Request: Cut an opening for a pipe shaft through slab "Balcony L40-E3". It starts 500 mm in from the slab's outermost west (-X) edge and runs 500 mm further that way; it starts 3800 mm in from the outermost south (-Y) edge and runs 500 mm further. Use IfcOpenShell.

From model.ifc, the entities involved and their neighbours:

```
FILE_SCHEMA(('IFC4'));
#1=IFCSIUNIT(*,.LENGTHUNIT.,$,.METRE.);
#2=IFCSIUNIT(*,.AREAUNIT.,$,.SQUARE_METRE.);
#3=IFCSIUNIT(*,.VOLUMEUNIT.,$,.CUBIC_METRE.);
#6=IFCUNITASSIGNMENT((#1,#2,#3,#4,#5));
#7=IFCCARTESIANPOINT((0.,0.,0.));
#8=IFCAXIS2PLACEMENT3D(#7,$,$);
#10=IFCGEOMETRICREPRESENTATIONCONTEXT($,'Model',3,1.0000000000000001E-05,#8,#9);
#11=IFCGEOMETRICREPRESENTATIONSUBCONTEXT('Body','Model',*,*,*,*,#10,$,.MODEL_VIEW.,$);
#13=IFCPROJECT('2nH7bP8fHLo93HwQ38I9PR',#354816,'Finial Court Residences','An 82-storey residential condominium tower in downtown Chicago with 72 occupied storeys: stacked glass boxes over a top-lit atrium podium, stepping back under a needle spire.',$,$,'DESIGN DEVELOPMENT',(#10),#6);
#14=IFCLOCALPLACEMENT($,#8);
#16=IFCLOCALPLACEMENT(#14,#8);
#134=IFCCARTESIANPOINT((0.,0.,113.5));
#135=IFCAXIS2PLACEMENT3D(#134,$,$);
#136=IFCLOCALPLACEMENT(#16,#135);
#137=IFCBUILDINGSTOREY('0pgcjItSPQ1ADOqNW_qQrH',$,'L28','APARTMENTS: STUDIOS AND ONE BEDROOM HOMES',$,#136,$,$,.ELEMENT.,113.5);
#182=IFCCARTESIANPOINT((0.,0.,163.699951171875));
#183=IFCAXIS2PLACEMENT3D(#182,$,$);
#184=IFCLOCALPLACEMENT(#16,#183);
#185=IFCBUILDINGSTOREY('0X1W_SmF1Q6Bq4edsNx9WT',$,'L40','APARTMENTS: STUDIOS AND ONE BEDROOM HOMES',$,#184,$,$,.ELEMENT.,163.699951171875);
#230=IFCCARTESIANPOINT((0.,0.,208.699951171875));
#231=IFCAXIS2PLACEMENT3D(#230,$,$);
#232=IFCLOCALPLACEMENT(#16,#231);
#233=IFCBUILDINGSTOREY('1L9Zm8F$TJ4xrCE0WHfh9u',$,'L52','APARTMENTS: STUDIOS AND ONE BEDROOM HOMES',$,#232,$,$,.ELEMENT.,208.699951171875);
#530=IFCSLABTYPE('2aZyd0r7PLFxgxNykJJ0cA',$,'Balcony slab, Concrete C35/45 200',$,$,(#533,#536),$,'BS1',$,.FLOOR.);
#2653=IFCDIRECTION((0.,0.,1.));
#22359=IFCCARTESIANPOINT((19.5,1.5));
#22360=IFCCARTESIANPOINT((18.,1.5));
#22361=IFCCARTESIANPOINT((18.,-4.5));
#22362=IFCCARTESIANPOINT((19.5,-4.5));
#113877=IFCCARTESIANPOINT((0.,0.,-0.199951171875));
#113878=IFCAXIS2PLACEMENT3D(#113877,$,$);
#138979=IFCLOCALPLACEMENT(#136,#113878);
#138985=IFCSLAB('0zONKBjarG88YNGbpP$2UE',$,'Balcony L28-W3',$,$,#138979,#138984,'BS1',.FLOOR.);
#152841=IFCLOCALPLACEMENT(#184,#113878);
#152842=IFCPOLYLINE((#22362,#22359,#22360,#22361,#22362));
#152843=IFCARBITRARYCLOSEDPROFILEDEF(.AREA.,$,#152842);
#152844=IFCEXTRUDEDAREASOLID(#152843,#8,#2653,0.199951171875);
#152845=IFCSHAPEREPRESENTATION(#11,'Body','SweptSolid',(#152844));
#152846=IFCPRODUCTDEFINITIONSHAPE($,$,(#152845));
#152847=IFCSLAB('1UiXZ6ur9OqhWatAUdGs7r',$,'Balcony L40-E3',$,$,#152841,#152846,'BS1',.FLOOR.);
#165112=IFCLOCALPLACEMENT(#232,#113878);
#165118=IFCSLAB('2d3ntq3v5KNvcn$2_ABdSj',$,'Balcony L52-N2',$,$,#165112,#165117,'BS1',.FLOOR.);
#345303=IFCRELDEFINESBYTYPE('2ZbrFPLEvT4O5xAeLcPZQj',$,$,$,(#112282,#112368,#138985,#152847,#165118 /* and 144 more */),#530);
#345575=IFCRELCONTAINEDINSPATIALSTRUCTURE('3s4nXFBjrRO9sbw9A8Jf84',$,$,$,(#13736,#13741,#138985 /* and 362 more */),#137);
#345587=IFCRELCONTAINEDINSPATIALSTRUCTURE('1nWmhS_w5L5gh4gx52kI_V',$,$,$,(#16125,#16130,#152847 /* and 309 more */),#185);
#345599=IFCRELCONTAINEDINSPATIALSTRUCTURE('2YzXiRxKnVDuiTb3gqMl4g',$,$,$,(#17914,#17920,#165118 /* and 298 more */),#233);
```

```python
import numpy as np
import ifcopenshell
import ifcopenshell.api.feature
import ifcopenshell.api.geometry
import ifcopenshell.api.root
import ifcopenshell.geom
import ifcopenshell.util.placement
import ifcopenshell.util.representation
import ifcopenshell.util.shape
import ifcopenshell.util.unit

model = ifcopenshell.open("model.ifc")
unit_scale = ifcopenshell.util.unit.calculate_unit_scale(model)
settings = ifcopenshell.geom.settings()


def volume(element):
    """Net volume in cubic metres, openings subtracted."""
    shape = ifcopenshell.geom.create_shape(settings, element)
    return ifcopenshell.util.shape.get_volume(shape.geometry)


slab = model.by_guid("1UiXZ6ur9OqhWatAUdGs7r")
before = volume(slab)

# Extent in the slab's own axes, in metres. The edges named are its -X and -Y sides.
slab_shape = ifcopenshell.geom.create_shape(settings, slab)
vertices = ifcopenshell.util.shape.get_vertices(slab_shape.geometry)
x_min, y_min, bottom = vertices.min(axis=0)
top = vertices[:, 2].max()

opening = ifcopenshell.api.root.create_entity(model, ifc_class="IfcOpeningElement", name="Pipe shaft opening", predefined_type="OPENING")
context = ifcopenshell.util.representation.get_context(model, "Model", "Body", "MODEL_VIEW")
width, depth = 0.5, 0.5
outline = [(0.0, 0.0), (width, 0.0), (width, depth), (0.0, depth), (0.0, 0.0)]
# Overshoot both faces by 50 mm so the cut is clean.
shape = ifcopenshell.api.geometry.add_slab_representation(
    model, context=context, depth=top - bottom + 0.1, polyline=outline
)
ifcopenshell.api.geometry.assign_representation(model, product=opening, representation=shape)

matrix = ifcopenshell.util.placement.get_local_placement(slab.ObjectPlacement)
matrix[:, 3] = matrix @ np.append(np.array([x_min + 0.5, y_min + 3.8, bottom - 0.05]) / unit_scale, 1.0)
ifcopenshell.api.geometry.edit_object_placement(model, product=opening, matrix=matrix, is_si=False)
ifcopenshell.api.feature.add_feature(model, feature=opening, element=slab)

after = volume(slab)

print(f"slab volume {before:.3f} -> {after:.3f} m3")

model.write("model_rev.ifc")
```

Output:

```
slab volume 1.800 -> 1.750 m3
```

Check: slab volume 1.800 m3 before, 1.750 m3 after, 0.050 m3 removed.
